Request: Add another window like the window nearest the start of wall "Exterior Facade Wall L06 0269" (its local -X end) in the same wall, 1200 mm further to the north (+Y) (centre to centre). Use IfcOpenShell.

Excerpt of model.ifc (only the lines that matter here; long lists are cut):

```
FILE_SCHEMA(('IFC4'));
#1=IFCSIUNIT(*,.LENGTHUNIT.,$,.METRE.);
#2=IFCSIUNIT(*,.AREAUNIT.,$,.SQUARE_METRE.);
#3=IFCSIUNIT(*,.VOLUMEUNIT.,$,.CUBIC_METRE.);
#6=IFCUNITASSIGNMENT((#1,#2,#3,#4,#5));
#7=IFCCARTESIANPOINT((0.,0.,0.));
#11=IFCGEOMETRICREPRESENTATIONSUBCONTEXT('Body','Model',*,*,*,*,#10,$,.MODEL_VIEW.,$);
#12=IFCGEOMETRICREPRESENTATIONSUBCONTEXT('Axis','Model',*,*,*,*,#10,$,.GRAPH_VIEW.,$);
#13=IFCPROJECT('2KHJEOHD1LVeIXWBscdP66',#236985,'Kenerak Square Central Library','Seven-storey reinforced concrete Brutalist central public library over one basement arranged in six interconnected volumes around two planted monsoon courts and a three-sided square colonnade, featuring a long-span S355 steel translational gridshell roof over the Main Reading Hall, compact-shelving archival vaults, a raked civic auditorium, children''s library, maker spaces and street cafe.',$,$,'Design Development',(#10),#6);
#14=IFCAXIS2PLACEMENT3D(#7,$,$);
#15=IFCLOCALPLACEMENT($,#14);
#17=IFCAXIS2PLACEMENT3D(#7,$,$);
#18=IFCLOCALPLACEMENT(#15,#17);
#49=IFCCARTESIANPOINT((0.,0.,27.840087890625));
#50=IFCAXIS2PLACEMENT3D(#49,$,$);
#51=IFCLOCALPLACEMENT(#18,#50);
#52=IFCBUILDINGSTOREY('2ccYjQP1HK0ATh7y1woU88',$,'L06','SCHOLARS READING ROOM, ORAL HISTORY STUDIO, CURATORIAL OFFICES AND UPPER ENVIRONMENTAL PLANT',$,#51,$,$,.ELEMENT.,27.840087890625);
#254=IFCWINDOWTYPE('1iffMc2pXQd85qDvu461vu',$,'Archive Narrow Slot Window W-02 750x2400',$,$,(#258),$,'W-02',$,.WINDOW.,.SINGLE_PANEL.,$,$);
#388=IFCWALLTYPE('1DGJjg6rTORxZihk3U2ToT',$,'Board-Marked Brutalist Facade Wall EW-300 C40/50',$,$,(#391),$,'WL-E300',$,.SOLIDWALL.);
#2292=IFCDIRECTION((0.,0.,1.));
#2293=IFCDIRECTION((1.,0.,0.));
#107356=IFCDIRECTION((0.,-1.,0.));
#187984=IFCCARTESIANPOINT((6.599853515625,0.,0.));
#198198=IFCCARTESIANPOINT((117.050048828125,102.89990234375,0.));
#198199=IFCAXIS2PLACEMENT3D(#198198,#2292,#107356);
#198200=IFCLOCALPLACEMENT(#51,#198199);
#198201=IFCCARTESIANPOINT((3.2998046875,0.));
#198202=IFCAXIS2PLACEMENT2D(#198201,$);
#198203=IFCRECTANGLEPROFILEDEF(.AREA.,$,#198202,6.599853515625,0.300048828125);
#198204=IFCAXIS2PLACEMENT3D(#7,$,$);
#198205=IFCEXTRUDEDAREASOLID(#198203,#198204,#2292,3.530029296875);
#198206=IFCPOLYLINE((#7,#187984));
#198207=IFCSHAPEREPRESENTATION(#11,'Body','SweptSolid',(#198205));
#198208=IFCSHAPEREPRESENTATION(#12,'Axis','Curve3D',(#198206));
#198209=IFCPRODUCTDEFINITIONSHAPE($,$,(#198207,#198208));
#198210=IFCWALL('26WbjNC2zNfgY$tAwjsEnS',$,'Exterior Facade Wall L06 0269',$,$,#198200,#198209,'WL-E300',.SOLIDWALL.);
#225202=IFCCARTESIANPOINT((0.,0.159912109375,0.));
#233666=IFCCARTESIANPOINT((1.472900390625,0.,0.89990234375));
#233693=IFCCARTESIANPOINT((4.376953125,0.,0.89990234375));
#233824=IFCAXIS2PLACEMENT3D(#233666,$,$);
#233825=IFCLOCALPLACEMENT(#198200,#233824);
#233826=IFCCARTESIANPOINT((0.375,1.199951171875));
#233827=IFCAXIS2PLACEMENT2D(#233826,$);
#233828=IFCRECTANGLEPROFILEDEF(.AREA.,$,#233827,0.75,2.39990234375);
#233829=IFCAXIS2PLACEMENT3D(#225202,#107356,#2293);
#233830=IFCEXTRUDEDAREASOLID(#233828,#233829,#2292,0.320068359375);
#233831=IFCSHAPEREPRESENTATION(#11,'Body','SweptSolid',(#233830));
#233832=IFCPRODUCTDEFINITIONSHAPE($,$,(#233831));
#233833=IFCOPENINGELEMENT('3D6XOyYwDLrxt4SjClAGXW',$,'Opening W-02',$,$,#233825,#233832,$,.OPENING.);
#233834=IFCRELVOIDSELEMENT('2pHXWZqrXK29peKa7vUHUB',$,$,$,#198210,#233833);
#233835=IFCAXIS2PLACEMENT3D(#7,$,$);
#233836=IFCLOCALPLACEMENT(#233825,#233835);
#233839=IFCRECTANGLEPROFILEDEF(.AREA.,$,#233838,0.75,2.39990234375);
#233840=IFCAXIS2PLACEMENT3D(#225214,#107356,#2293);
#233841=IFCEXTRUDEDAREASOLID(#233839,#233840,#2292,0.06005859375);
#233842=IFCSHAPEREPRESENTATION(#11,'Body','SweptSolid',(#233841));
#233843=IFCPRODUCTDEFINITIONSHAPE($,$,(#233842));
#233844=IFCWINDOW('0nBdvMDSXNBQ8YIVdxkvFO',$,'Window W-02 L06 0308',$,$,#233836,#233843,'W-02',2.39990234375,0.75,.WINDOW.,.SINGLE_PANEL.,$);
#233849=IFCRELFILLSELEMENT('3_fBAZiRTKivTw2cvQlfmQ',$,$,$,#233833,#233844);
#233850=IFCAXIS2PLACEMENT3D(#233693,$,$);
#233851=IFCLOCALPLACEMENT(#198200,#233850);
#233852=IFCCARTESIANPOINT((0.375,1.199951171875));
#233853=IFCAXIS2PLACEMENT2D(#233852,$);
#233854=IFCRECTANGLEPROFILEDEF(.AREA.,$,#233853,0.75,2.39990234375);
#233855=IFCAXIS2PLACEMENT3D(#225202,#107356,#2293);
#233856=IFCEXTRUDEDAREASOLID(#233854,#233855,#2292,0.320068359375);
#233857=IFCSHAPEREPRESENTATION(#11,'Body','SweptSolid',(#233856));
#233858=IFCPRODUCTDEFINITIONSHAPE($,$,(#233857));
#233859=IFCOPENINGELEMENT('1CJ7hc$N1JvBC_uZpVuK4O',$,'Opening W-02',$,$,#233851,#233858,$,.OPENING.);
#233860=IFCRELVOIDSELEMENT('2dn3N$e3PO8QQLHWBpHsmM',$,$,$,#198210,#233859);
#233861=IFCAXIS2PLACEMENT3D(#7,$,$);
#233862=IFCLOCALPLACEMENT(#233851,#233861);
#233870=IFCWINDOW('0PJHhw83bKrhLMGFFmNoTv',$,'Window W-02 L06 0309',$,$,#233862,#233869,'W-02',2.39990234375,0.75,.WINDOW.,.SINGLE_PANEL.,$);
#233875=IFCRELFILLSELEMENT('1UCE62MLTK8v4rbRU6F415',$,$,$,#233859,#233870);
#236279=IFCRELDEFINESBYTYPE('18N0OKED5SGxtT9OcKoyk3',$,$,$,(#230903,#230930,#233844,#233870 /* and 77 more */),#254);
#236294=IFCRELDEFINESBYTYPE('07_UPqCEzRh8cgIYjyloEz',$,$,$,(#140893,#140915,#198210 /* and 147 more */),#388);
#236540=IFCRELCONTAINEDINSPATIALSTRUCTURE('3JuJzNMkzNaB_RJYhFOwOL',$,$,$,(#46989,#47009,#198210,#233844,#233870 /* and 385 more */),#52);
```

```python
import ifcopenshell
import ifcopenshell.api.feature
import ifcopenshell.api.geometry
import ifcopenshell.api.root
import ifcopenshell.geom
import ifcopenshell.util.element
import ifcopenshell.util.placement
import ifcopenshell.util.shape
import ifcopenshell.util.unit

model = ifcopenshell.open("model.ifc")
unit_scale = ifcopenshell.util.unit.calculate_unit_scale(model)
settings = ifcopenshell.geom.settings()


def volume(element):
    """Net volume in cubic metres, openings subtracted."""
    shape = ifcopenshell.geom.create_shape(settings, element)
    return ifcopenshell.util.shape.get_volume(shape.geometry)


window = model.by_id(233844)
opening = window.FillsVoids[0].RelatingOpeningElement
wall = opening.VoidsElements[0].RelatingBuildingElement
before = volume(wall)
shift = ifcopenshell.util.placement.get_local_placement(wall.ObjectPlacement)[:3, 0] * -1.2 / unit_scale

# copy_class copies the void relationship, type, container and properties, but no geometry.
new_opening = ifcopenshell.api.root.copy_class(model, product=opening)
new_opening.Representation = ifcopenshell.util.element.copy_deep(
    model, opening.Representation, exclude=["IfcGeometricRepresentationContext", "IfcRepresentationMap"]
)
new_window = ifcopenshell.api.root.copy_class(model, product=window)
new_window.Representation = ifcopenshell.util.element.copy_deep(
    model, window.Representation, exclude=["IfcGeometricRepresentationContext", "IfcRepresentationMap"]
)
new_window.Tag = None
ifcopenshell.api.feature.add_filling(model, opening=new_opening, element=new_window)

for old, new in ((opening, new_opening), (window, new_window)):
    matrix = ifcopenshell.util.placement.get_local_placement(old.ObjectPlacement)
    matrix[:3, 3] += shift
    ifcopenshell.api.geometry.edit_object_placement(model, product=new, matrix=matrix, is_si=False)

after = volume(wall)

print(f"wall volume {before:.3f} -> {after:.3f} m3")

model.write("model_v2.ifc")
```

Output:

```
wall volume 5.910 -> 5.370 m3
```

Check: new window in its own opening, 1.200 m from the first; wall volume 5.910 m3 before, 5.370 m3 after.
